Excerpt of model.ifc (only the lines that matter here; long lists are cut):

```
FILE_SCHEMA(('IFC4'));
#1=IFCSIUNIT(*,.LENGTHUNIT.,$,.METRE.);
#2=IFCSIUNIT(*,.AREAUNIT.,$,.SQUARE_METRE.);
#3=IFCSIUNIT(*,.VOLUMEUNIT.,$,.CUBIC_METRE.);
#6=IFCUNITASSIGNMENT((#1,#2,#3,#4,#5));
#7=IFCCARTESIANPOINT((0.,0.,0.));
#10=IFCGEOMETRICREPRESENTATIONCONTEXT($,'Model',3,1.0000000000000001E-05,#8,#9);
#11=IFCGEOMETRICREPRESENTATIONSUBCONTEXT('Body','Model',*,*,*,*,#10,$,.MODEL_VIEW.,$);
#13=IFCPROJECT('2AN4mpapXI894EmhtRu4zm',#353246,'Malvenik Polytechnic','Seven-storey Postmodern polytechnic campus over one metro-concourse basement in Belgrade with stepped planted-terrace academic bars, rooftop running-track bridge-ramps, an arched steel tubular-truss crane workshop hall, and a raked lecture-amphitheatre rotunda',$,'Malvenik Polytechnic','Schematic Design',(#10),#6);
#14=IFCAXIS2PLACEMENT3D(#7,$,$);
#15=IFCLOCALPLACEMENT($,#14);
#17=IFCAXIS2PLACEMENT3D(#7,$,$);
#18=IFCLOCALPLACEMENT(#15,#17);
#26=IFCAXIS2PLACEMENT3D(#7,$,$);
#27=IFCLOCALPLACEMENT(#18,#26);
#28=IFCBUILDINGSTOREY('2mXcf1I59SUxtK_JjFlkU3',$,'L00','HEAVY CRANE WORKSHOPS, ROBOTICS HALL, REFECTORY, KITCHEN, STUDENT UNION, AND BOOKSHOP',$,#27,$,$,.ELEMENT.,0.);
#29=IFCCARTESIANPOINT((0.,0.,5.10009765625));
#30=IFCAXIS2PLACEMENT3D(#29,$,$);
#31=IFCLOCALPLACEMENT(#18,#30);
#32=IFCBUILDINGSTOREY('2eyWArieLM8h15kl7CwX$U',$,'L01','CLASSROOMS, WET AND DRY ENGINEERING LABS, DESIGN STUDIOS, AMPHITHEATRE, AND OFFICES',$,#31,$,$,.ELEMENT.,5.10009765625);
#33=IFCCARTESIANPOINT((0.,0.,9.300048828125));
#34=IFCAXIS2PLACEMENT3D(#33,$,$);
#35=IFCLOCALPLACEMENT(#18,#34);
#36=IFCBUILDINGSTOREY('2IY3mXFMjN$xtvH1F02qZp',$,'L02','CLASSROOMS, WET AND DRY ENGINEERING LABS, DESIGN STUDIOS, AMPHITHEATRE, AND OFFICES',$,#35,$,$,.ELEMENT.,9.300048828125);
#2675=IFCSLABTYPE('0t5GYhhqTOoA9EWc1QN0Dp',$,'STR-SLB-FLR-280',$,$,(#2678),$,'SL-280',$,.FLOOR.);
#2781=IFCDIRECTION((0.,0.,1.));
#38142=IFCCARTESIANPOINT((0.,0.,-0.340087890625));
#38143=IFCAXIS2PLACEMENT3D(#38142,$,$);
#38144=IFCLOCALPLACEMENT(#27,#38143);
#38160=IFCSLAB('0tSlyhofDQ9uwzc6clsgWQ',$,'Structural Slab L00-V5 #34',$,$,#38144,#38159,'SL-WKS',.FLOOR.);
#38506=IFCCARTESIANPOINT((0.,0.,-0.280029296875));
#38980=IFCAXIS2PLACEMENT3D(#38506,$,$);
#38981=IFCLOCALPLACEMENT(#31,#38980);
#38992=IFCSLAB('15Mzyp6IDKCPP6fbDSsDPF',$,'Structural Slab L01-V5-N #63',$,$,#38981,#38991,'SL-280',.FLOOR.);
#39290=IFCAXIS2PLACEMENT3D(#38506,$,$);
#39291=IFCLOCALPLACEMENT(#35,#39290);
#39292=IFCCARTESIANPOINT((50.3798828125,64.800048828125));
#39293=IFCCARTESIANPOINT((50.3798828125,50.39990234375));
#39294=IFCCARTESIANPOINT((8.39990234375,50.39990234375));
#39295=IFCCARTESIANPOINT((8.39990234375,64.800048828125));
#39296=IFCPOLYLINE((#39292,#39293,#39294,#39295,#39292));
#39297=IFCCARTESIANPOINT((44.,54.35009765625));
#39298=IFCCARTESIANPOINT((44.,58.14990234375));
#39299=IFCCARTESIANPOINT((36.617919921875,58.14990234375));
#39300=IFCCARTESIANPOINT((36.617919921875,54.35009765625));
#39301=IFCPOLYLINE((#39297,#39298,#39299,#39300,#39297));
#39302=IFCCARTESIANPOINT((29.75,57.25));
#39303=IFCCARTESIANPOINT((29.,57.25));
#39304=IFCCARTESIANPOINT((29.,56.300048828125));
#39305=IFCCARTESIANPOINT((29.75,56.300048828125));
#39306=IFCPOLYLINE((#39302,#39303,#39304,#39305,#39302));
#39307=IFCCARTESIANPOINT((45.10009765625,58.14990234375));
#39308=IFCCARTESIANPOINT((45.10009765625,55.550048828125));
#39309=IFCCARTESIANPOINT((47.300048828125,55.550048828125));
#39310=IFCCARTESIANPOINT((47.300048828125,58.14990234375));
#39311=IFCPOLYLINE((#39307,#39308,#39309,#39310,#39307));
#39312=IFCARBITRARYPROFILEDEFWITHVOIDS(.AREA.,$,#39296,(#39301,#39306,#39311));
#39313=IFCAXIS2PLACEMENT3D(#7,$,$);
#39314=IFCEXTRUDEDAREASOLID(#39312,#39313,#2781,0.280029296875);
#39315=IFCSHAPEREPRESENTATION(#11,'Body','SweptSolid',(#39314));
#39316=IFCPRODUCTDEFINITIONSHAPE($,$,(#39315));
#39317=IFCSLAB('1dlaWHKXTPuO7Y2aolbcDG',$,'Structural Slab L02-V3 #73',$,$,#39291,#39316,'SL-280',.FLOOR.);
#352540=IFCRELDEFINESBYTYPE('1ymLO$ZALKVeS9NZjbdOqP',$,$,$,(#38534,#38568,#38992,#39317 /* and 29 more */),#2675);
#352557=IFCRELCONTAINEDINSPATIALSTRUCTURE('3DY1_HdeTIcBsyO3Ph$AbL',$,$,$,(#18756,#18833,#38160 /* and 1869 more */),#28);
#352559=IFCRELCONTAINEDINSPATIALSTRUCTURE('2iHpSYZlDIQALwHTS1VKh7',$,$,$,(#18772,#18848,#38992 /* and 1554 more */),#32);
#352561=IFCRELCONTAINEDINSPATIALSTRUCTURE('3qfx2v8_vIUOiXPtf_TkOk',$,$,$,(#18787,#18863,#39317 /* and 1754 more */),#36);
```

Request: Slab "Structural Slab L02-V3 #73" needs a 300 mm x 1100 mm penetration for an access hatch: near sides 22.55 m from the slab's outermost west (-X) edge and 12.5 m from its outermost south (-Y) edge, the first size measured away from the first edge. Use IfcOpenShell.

```python
import numpy as np
import ifcopenshell
import ifcopenshell.api.feature
import ifcopenshell.api.geometry
import ifcopenshell.api.root
import ifcopenshell.geom
import ifcopenshell.util.placement
import ifcopenshell.util.representation
import ifcopenshell.util.shape
import ifcopenshell.util.unit

model = ifcopenshell.open("model.ifc")
unit_scale = ifcopenshell.util.unit.calculate_unit_scale(model)
settings = ifcopenshell.geom.settings()


def volume(element):
    """Net volume in cubic metres, openings subtracted."""
    shape = ifcopenshell.geom.create_shape(settings, element)
    return ifcopenshell.util.shape.get_volume(shape.geometry)


slab = model.by_id(39317)
before = volume(slab)

# Extent in the slab's own axes, in metres. The edges named are its -X and -Y sides.
slab_shape = ifcopenshell.geom.create_shape(settings, slab)
vertices = ifcopenshell.util.shape.get_vertices(slab_shape.geometry)
x_min, y_min, bottom = vertices.min(axis=0)
top = vertices[:, 2].max()

opening = ifcopenshell.api.root.create_entity(model, ifc_class="IfcOpeningElement", name="Access hatch opening", predefined_type="OPENING")
context = ifcopenshell.util.representation.get_context(model, "Model", "Body", "MODEL_VIEW")
width, depth = 0.3, 1.1
outline = [(0.0, 0.0), (width, 0.0), (width, depth), (0.0, depth), (0.0, 0.0)]
# Overshoot both faces by 50 mm so the cut is clean.
shape = ifcopenshell.api.geometry.add_slab_representation(
    model, context=context, depth=top - bottom + 0.1, polyline=outline
)
ifcopenshell.api.geometry.assign_representation(model, product=opening, representation=shape)

matrix = ifcopenshell.util.placement.get_local_placement(slab.ObjectPlacement)
matrix[:, 3] = matrix @ np.append(np.array([x_min + 22.55, y_min + 12.5, bottom - 0.05]) / unit_scale, 1.0)
ifcopenshell.api.geometry.edit_object_placement(model, product=opening, matrix=matrix, is_si=False)
ifcopenshell.api.feature.add_feature(model, feature=opening, element=slab)

after = volume(slab)

print(f"slab volume {before:.3f} -> {after:.3f} m3")

model.write("model_rev.ifc")
```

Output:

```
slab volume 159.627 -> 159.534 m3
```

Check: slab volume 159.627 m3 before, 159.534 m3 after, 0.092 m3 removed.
